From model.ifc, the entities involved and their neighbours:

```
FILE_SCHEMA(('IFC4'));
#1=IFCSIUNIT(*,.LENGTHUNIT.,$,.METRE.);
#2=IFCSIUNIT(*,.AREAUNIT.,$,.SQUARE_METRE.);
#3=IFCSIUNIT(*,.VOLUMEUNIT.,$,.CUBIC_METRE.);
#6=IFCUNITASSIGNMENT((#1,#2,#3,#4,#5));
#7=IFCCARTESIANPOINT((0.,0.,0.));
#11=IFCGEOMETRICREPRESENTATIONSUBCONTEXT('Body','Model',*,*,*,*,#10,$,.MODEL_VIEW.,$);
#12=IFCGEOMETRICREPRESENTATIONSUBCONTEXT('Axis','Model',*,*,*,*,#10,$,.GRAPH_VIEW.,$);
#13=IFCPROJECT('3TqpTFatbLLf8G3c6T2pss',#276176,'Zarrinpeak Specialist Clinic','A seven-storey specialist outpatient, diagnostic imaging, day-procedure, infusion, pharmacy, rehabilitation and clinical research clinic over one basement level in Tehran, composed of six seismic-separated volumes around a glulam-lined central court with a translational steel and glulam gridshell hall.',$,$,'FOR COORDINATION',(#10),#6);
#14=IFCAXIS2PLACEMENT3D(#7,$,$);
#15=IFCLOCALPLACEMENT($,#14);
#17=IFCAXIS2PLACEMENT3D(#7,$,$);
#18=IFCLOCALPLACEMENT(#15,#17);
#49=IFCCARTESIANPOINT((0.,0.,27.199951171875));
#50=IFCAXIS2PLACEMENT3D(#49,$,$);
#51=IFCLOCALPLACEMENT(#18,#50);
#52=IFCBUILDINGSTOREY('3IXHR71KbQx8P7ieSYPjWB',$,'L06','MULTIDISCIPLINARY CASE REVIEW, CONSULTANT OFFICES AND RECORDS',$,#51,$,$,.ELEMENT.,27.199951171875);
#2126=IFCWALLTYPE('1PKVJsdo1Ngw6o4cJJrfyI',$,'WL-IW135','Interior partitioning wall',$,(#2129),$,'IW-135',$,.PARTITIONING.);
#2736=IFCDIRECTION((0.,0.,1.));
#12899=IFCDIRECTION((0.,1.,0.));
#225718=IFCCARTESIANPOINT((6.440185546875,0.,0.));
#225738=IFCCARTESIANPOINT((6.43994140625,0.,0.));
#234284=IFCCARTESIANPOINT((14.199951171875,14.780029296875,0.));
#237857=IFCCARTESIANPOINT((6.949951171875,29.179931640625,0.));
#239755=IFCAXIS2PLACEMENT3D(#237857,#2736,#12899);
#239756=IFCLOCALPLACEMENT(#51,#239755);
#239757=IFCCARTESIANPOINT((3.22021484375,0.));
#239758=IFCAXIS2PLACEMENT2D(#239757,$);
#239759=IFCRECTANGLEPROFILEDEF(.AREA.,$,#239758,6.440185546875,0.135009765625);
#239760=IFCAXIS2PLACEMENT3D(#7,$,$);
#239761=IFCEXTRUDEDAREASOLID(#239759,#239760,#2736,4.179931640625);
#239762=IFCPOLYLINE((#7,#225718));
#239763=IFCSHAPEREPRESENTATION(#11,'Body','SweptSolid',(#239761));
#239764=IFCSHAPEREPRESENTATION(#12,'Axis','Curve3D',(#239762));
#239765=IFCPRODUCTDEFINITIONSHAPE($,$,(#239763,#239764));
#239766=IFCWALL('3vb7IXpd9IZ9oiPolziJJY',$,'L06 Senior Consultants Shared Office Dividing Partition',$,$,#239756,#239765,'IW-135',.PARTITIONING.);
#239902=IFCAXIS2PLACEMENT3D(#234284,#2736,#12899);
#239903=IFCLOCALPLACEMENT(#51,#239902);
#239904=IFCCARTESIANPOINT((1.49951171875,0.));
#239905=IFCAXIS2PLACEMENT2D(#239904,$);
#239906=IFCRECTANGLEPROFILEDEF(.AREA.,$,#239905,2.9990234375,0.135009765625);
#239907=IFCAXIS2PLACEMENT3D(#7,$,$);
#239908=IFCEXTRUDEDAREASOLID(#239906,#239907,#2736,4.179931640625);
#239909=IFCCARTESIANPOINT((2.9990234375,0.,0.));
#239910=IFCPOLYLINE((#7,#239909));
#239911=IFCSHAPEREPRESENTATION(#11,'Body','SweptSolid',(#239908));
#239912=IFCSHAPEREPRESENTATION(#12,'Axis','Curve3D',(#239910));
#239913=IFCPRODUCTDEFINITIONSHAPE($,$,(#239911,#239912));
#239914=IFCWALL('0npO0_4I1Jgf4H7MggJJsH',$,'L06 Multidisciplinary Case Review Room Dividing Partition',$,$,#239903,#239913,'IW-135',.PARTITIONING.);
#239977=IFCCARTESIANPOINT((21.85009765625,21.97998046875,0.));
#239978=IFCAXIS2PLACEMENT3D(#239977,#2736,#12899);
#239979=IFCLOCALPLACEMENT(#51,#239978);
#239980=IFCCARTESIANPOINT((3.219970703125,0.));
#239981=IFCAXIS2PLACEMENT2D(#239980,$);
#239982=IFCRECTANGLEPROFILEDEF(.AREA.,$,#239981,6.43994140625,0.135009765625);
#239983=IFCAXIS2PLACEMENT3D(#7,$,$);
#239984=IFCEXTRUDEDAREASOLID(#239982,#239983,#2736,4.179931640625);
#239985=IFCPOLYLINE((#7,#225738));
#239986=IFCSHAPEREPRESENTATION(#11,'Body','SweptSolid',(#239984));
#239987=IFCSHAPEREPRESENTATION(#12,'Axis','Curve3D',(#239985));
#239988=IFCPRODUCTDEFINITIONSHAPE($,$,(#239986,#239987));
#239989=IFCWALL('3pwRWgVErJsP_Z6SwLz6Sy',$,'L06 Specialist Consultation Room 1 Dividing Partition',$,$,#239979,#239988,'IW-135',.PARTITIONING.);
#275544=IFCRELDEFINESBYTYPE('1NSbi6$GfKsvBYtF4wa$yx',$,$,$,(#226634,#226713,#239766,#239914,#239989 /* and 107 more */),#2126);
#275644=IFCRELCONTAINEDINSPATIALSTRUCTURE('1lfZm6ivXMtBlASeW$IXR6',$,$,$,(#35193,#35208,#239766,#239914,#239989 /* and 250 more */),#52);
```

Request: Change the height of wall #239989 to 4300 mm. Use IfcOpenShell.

```python
import ifcopenshell
import ifcopenshell.geom
import ifcopenshell.util.representation
import ifcopenshell.util.shape
import ifcopenshell.util.unit

model = ifcopenshell.open("model.ifc")
unit_scale = ifcopenshell.util.unit.calculate_unit_scale(model)
settings = ifcopenshell.geom.settings()


def volume(element):
    """Net volume in cubic metres, openings subtracted."""
    shape = ifcopenshell.geom.create_shape(settings, element)
    return ifcopenshell.util.shape.get_volume(shape.geometry)


wall = model.by_id(239989)
before = volume(wall)

body = ifcopenshell.util.representation.get_representation(wall, "Model", "Body")
solid = body.Items[0]
old_height = solid.Depth
solid.Depth = 4.3 / unit_scale
after = volume(wall)

print(f"height {old_height:g} -> {solid.Depth:g}, volume {before:.3f} -> {after:.3f} m3")

model.write("model_updated.ifc")
```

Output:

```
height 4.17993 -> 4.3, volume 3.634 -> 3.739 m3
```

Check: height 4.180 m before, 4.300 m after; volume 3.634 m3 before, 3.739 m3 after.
